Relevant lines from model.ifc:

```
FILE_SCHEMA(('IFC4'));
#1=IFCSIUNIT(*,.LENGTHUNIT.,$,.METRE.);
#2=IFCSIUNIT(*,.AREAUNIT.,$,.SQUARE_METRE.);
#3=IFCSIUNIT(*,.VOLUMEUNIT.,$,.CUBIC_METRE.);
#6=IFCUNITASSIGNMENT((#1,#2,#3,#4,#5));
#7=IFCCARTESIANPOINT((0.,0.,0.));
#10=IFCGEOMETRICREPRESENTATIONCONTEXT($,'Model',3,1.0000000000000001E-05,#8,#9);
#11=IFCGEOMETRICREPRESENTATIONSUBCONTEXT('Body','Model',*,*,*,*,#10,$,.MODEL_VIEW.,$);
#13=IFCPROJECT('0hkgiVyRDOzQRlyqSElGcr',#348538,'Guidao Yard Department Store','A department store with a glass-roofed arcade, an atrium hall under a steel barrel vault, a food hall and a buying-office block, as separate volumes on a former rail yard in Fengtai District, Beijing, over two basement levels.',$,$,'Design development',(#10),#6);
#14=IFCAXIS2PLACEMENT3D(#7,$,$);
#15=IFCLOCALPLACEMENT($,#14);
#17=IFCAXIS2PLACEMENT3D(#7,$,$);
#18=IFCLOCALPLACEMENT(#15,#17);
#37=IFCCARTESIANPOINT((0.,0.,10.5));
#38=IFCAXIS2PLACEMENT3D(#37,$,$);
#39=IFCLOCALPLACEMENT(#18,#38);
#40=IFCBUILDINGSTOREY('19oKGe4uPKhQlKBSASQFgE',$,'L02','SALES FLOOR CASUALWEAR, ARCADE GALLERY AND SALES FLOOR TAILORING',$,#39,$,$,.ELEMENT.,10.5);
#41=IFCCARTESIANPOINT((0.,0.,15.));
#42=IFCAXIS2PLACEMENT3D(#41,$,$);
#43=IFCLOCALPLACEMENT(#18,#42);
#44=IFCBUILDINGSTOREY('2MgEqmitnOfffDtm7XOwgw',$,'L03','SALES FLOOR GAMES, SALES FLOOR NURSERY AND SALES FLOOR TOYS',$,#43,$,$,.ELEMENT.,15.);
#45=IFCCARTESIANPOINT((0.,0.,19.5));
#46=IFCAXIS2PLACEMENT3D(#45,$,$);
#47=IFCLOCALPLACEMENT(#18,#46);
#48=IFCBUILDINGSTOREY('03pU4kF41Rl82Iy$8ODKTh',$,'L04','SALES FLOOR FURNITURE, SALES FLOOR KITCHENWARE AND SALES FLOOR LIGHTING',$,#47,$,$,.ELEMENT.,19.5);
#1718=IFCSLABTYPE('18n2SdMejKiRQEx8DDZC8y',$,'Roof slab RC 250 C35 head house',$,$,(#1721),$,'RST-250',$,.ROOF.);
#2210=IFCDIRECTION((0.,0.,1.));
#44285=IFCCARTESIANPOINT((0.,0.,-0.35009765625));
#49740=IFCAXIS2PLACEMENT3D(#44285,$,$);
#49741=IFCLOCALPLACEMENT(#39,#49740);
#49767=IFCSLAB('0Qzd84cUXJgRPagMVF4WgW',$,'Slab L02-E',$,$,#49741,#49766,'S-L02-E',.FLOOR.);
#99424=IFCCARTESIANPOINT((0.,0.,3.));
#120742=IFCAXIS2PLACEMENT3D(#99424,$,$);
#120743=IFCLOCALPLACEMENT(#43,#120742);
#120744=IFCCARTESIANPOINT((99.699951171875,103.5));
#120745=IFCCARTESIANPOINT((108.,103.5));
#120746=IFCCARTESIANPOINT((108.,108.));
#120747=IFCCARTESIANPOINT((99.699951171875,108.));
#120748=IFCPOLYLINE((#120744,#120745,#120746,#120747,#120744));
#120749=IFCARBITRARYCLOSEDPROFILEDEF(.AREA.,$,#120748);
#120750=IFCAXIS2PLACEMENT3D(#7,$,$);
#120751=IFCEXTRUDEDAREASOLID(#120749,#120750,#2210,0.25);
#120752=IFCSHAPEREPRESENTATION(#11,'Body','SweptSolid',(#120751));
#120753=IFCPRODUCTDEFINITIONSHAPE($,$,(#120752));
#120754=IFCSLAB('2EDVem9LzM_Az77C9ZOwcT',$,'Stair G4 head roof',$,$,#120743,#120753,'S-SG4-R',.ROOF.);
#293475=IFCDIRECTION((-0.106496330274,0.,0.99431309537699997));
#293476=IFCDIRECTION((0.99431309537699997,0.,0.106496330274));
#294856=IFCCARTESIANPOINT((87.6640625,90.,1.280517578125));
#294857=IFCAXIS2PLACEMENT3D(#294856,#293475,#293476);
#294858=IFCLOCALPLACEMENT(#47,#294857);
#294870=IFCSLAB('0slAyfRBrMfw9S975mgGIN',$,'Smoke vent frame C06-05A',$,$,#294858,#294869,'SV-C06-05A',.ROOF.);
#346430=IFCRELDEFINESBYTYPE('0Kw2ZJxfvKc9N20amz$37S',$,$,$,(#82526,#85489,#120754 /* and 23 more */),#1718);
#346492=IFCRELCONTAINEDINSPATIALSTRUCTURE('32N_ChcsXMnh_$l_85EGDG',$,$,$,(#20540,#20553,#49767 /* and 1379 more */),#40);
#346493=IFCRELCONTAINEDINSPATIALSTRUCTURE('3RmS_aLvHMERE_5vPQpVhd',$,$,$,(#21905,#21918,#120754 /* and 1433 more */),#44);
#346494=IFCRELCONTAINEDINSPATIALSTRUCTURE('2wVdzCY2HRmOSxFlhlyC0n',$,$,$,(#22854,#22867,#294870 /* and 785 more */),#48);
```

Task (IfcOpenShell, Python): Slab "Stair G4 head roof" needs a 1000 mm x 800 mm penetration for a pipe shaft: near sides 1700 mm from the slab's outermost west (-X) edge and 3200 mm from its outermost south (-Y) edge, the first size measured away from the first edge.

```python
import numpy as np
import ifcopenshell
import ifcopenshell.api.feature
import ifcopenshell.api.geometry
import ifcopenshell.api.root
import ifcopenshell.geom
import ifcopenshell.util.placement
import ifcopenshell.util.representation
import ifcopenshell.util.shape
import ifcopenshell.util.unit

model = ifcopenshell.open("model.ifc")
unit_scale = ifcopenshell.util.unit.calculate_unit_scale(model)
settings = ifcopenshell.geom.settings()


def volume(element):
    """Net volume in cubic metres, openings subtracted."""
    shape = ifcopenshell.geom.create_shape(settings, element)
    return ifcopenshell.util.shape.get_volume(shape.geometry)


slab = model.by_guid("2EDVem9LzM_Az77C9ZOwcT")
before = volume(slab)

# Extent in the slab's own axes, in metres. The edges named are its -X and -Y sides.
slab_shape = ifcopenshell.geom.create_shape(settings, slab)
vertices = ifcopenshell.util.shape.get_vertices(slab_shape.geometry)
x_min, y_min, bottom = vertices.min(axis=0)
top = vertices[:, 2].max()

opening = ifcopenshell.api.root.create_entity(model, ifc_class="IfcOpeningElement", name="Pipe shaft opening", predefined_type="OPENING")
context = ifcopenshell.util.representation.get_context(model, "Model", "Body", "MODEL_VIEW")
width, depth = 1, 0.8
outline = [(0.0, 0.0), (width, 0.0), (width, depth), (0.0, depth), (0.0, 0.0)]
# Overshoot both faces by 50 mm so the cut is clean.
shape = ifcopenshell.api.geometry.add_slab_representation(
    model, context=context, depth=top - bottom + 0.1, polyline=outline
)
ifcopenshell.api.geometry.assign_representation(model, product=opening, representation=shape)

matrix = ifcopenshell.util.placement.get_local_placement(slab.ObjectPlacement)
matrix[:, 3] = matrix @ np.append(np.array([x_min + 1.7, y_min + 3.2, bottom - 0.05]) / unit_scale, 1.0)
ifcopenshell.api.geometry.edit_object_placement(model, product=opening, matrix=matrix, is_si=False)
ifcopenshell.api.feature.add_feature(model, feature=opening, element=slab)

after = volume(slab)

print(f"slab volume {before:.3f} -> {after:.3f} m3")

model.write("model_rev.ifc")
```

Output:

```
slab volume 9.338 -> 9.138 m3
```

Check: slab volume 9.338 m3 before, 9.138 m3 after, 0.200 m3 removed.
